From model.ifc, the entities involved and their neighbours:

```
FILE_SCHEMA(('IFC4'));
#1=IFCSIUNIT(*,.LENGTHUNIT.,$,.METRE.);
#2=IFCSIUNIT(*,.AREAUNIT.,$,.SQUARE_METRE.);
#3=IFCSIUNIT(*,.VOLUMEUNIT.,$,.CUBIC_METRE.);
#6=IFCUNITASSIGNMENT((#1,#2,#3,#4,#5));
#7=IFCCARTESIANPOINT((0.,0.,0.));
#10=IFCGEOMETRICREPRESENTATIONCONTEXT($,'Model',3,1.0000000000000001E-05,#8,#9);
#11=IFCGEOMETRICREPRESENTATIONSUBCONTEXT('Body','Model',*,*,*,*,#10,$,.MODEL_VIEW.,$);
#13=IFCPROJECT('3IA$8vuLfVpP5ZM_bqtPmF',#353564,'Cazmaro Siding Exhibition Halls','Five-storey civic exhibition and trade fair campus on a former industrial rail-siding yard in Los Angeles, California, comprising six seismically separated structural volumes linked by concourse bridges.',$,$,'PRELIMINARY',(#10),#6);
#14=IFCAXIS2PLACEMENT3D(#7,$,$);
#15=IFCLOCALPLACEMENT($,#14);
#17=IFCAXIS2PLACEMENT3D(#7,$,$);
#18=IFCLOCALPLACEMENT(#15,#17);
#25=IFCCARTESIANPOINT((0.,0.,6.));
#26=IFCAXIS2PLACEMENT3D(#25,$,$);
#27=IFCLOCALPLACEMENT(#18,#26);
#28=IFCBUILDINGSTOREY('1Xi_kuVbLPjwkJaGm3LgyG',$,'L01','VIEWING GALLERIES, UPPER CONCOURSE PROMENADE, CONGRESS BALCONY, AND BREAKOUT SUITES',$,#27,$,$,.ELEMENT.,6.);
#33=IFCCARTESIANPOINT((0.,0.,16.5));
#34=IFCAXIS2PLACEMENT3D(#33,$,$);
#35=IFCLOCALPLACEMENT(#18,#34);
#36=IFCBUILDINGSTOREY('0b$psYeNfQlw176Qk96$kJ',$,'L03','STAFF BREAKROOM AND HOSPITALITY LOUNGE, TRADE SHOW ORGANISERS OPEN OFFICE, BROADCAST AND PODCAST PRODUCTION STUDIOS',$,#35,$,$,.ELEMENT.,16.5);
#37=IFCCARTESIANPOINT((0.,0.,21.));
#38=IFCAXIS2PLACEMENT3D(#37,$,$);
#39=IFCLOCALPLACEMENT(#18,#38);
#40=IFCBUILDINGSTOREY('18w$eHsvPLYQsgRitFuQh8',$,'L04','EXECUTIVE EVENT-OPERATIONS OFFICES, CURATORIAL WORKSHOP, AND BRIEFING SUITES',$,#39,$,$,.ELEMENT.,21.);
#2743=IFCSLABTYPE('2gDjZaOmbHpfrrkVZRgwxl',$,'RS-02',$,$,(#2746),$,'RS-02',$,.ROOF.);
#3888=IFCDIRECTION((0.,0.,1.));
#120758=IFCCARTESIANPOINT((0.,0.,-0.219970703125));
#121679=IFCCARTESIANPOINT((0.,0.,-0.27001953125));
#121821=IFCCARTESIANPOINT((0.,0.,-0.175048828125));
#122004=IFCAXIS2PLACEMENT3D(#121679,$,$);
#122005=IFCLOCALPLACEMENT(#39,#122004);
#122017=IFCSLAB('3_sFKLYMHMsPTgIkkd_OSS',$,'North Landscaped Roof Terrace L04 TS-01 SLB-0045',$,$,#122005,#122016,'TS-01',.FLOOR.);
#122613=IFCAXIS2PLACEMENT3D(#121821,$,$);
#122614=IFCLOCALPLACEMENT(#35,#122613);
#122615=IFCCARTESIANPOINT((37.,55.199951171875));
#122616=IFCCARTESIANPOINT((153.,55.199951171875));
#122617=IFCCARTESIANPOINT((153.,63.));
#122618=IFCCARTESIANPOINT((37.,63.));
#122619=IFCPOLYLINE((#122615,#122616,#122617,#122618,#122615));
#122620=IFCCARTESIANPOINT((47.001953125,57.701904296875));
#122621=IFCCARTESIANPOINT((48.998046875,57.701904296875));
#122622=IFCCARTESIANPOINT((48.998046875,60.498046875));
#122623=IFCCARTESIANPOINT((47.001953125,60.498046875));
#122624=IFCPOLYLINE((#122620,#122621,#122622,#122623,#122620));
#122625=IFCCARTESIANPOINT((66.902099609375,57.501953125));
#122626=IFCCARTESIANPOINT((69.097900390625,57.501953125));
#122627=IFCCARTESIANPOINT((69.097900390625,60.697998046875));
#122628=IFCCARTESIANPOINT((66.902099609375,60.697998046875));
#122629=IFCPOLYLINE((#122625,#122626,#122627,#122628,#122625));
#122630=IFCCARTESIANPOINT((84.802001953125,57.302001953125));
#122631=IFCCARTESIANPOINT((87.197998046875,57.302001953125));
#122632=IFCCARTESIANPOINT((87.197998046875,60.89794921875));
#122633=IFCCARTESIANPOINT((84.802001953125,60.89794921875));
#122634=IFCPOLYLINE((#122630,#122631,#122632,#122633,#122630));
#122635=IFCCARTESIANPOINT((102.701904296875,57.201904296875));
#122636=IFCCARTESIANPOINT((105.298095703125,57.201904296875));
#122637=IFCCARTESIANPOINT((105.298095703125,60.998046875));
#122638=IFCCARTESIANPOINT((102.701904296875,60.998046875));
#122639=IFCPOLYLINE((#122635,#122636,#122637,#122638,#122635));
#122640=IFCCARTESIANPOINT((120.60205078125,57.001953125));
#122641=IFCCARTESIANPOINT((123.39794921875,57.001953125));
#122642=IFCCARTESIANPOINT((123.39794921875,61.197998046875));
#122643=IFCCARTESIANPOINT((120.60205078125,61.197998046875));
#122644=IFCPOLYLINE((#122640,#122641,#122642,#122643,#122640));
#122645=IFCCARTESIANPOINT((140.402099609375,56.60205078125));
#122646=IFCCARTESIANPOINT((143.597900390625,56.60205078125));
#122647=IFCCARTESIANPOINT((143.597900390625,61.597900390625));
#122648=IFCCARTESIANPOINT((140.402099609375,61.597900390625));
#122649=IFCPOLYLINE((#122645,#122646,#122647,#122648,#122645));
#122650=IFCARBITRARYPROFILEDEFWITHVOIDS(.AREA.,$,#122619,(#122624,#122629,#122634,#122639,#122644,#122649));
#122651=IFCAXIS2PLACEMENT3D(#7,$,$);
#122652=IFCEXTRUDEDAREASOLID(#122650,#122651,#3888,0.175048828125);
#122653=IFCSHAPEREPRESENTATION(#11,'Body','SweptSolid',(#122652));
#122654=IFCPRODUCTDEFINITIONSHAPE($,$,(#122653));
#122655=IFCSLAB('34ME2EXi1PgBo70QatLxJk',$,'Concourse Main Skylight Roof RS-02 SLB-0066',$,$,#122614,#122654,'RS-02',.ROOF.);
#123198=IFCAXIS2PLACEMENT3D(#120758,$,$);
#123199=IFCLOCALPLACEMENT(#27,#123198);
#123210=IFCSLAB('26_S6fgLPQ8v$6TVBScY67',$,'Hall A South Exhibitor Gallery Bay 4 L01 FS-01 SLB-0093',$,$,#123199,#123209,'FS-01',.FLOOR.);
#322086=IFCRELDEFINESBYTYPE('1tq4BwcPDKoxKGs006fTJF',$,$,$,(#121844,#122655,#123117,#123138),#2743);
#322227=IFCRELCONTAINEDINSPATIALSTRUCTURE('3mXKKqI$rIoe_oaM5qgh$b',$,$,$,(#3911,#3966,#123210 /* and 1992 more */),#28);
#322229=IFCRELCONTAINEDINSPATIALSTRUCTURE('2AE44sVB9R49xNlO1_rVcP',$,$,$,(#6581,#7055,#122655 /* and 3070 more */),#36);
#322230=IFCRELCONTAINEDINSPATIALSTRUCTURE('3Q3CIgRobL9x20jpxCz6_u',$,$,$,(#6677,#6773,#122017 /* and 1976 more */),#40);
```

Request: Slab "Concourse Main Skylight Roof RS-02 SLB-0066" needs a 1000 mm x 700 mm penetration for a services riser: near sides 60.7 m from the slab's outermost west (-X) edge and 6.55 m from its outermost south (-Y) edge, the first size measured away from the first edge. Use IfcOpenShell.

```python
import numpy as np
import ifcopenshell
import ifcopenshell.api.feature
import ifcopenshell.api.geometry
import ifcopenshell.api.root
import ifcopenshell.geom
import ifcopenshell.util.placement
import ifcopenshell.util.representation
import ifcopenshell.util.shape
import ifcopenshell.util.unit

model = ifcopenshell.open("model.ifc")
unit_scale = ifcopenshell.util.unit.calculate_unit_scale(model)
settings = ifcopenshell.geom.settings()


def volume(element):
    """Net volume in cubic metres, openings subtracted."""
    shape = ifcopenshell.geom.create_shape(settings, element)
    return ifcopenshell.util.shape.get_volume(shape.geometry)


slab = model.by_guid("34ME2EXi1PgBo70QatLxJk")
before = volume(slab)

# Extent in the slab's own axes, in metres. The edges named are its -X and -Y sides.
slab_shape = ifcopenshell.geom.create_shape(settings, slab)
vertices = ifcopenshell.util.shape.get_vertices(slab_shape.geometry)
x_min, y_min, bottom = vertices.min(axis=0)
top = vertices[:, 2].max()

opening = ifcopenshell.api.root.create_entity(model, ifc_class="IfcOpeningElement", name="Services riser opening", predefined_type="OPENING")
context = ifcopenshell.util.representation.get_context(model, "Model", "Body", "MODEL_VIEW")
width, depth = 1, 0.7
outline = [(0.0, 0.0), (width, 0.0), (width, depth), (0.0, depth), (0.0, 0.0)]
# Overshoot both faces by 50 mm so the cut is clean.
shape = ifcopenshell.api.geometry.add_slab_representation(
    model, context=context, depth=top - bottom + 0.1, polyline=outline
)
ifcopenshell.api.geometry.assign_representation(model, product=opening, representation=shape)

matrix = ifcopenshell.util.placement.get_local_placement(slab.ObjectPlacement)
matrix[:, 3] = matrix @ np.append(np.array([x_min + 60.7, y_min + 6.55, bottom - 0.05]) / unit_scale, 1.0)
ifcopenshell.api.geometry.edit_object_placement(model, product=opening, matrix=matrix, is_si=False)
ifcopenshell.api.feature.add_feature(model, feature=opening, element=slab)

after = volume(slab)

print(f"slab volume {before:.3f} -> {after:.3f} m3")

model.write("model_updated.ifc")
```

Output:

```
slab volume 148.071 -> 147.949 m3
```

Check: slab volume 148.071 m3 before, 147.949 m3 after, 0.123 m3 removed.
